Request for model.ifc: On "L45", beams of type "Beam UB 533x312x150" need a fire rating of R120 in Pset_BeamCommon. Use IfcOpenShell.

First a look at what the model holds.

```python
import ifcopenshell
import ifcopenshell.util.element

model = ifcopenshell.open("model.ifc")
print(model.schema)
storey = next(s for s in model.by_type("IfcBuildingStorey") if s.Name == "L45")
beams = [e for e in ifcopenshell.util.element.get_decomposition(storey) if e.is_a("IfcBeam")]
seen = {}
for e in beams:
    element_type = ifcopenshell.util.element.get_type(e)
    key = (element_type.Name if element_type != e and element_type else None, ifcopenshell.util.element.get_pset(e, "Pset_BeamCommon", "FireRating"))
    seen[key] = seen.get(key, 0) + 1
for (name, value), count in sorted(seen.items(), key=str):
    print(count, "x", name, "|", value)
```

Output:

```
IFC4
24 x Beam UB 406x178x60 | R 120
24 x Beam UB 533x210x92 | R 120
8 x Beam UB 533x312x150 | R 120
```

```python
import ifcopenshell
import ifcopenshell.api.pset
import ifcopenshell.util.element

model = ifcopenshell.open("model.ifc")

storey = next(s for s in model.by_type("IfcBuildingStorey") if s.Name == "L45")
beams = [e for e in ifcopenshell.util.element.get_decomposition(storey) if e.is_a("IfcBeam")]

count = 0
for e in beams:
    element_type = ifcopenshell.util.element.get_type(e)
    if element_type in (None, e) or element_type.Name != "Beam UB 533x312x150":
        continue
    found = ifcopenshell.util.element.get_pset(e, "Pset_BeamCommon", should_inherit=False)
    if found:
        pset = model.by_id(found["id"])
        if len(ifcopenshell.util.element.get_elements_by_pset(pset)) > 1:
            pset = ifcopenshell.api.pset.unshare_pset(model, products=[e], pset=pset)[0]
    else:
        pset = ifcopenshell.api.pset.add_pset(model, product=e, name="Pset_BeamCommon")
    ifcopenshell.api.pset.edit_pset(model, pset=pset, properties={"FireRating": "R120"})
    count += 1

print(count, "beams updated")

model.write("model_edited.ifc")
```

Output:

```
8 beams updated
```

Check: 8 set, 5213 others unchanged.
